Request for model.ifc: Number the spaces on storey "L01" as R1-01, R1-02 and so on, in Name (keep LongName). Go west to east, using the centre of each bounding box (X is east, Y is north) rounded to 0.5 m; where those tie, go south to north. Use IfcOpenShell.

First a look at what the model holds.

```python
import ifcopenshell
import ifcopenshell.util.element
import ifcopenshell.util.placement

model = ifcopenshell.open("model.ifc")
print(model.schema)
storey = next(s for s in model.by_type("IfcBuildingStorey") if s.Name == "L01")
spaces = [e for e in ifcopenshell.util.element.get_decomposition(storey) if e.is_a("IfcSpace")]
for e in sorted(spaces, key=lambda e: e.id()):
    origin = ifcopenshell.util.placement.get_local_placement(e.ObjectPlacement)[:3, 3]
    print(e.id(), e.Name, e.LongName, origin.round(2) + 0.0, sep=" | ")
```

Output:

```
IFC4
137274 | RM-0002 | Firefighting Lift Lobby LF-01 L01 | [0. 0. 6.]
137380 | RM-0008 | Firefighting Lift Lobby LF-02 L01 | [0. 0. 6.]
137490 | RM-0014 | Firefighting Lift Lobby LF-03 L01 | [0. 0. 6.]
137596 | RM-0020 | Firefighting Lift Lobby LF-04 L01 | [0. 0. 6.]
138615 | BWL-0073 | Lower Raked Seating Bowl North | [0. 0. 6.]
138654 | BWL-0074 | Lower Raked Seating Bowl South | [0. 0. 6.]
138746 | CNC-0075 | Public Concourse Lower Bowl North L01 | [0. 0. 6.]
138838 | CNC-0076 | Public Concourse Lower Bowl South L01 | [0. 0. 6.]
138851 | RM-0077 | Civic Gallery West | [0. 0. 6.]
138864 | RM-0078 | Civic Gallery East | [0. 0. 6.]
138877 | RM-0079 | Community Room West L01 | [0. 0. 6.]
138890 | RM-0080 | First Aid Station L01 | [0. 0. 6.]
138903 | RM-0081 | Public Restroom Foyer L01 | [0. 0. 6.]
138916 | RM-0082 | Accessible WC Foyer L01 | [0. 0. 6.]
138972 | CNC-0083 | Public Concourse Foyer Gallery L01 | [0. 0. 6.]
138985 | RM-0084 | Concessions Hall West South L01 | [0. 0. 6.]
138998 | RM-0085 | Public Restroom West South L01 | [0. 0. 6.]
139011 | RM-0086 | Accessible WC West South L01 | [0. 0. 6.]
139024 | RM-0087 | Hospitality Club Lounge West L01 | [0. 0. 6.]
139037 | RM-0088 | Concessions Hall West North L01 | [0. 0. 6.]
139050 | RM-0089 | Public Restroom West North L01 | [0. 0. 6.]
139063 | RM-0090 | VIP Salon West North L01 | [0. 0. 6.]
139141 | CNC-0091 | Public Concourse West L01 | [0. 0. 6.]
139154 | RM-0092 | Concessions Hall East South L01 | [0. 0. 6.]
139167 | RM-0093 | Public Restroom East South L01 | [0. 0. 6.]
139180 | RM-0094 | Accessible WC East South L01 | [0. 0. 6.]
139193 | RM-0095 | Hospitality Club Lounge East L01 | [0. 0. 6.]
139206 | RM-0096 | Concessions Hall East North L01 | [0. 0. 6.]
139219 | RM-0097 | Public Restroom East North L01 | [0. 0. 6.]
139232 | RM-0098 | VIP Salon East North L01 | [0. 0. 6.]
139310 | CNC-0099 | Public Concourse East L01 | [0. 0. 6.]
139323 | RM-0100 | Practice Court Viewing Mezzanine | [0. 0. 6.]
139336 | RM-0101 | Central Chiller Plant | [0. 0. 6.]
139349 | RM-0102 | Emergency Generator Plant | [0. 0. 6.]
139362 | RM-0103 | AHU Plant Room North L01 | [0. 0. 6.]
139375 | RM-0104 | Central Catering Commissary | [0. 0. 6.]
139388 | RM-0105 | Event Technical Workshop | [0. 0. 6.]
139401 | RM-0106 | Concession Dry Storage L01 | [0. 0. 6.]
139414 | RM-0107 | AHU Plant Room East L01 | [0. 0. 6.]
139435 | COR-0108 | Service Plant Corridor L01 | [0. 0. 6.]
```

```python
import ifcopenshell
import ifcopenshell.geom
import ifcopenshell.util.element
import ifcopenshell.util.shape

model = ifcopenshell.open("model.ifc")
settings = ifcopenshell.geom.settings()
settings.set("use-world-coords", True)


def centre(element):
    shape = ifcopenshell.geom.create_shape(settings, element)
    return ifcopenshell.util.shape.get_bbox_centroid(shape.geometry)


storey = next(s for s in model.by_type("IfcBuildingStorey") if s.Name == "L01")
spaces = [e for e in ifcopenshell.util.element.get_decomposition(storey) if e.is_a("IfcSpace")]

# Insertion points can sit at a corner or the storey origin, so sort by the geometry (in metres).
centres = {e: centre(e) for e in spaces}
spaces.sort(key=lambda e: (round(centres[e][0] / 0.5), centres[e][1]))

for i, e in enumerate(spaces, start=1):
    number = f"R1-{i:02d}"
    e.Name = number
    print(e.id(), number)

model.write("model_edited.ifc")
```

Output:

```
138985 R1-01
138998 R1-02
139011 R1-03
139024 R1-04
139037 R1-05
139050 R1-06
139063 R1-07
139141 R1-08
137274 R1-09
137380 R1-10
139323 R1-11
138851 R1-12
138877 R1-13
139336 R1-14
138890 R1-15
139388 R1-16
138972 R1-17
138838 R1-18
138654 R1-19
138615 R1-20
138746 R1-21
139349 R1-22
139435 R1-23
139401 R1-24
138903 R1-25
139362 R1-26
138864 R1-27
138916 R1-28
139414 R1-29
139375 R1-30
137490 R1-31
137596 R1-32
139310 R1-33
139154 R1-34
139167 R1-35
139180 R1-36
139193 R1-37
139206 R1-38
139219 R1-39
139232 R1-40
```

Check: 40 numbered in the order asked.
